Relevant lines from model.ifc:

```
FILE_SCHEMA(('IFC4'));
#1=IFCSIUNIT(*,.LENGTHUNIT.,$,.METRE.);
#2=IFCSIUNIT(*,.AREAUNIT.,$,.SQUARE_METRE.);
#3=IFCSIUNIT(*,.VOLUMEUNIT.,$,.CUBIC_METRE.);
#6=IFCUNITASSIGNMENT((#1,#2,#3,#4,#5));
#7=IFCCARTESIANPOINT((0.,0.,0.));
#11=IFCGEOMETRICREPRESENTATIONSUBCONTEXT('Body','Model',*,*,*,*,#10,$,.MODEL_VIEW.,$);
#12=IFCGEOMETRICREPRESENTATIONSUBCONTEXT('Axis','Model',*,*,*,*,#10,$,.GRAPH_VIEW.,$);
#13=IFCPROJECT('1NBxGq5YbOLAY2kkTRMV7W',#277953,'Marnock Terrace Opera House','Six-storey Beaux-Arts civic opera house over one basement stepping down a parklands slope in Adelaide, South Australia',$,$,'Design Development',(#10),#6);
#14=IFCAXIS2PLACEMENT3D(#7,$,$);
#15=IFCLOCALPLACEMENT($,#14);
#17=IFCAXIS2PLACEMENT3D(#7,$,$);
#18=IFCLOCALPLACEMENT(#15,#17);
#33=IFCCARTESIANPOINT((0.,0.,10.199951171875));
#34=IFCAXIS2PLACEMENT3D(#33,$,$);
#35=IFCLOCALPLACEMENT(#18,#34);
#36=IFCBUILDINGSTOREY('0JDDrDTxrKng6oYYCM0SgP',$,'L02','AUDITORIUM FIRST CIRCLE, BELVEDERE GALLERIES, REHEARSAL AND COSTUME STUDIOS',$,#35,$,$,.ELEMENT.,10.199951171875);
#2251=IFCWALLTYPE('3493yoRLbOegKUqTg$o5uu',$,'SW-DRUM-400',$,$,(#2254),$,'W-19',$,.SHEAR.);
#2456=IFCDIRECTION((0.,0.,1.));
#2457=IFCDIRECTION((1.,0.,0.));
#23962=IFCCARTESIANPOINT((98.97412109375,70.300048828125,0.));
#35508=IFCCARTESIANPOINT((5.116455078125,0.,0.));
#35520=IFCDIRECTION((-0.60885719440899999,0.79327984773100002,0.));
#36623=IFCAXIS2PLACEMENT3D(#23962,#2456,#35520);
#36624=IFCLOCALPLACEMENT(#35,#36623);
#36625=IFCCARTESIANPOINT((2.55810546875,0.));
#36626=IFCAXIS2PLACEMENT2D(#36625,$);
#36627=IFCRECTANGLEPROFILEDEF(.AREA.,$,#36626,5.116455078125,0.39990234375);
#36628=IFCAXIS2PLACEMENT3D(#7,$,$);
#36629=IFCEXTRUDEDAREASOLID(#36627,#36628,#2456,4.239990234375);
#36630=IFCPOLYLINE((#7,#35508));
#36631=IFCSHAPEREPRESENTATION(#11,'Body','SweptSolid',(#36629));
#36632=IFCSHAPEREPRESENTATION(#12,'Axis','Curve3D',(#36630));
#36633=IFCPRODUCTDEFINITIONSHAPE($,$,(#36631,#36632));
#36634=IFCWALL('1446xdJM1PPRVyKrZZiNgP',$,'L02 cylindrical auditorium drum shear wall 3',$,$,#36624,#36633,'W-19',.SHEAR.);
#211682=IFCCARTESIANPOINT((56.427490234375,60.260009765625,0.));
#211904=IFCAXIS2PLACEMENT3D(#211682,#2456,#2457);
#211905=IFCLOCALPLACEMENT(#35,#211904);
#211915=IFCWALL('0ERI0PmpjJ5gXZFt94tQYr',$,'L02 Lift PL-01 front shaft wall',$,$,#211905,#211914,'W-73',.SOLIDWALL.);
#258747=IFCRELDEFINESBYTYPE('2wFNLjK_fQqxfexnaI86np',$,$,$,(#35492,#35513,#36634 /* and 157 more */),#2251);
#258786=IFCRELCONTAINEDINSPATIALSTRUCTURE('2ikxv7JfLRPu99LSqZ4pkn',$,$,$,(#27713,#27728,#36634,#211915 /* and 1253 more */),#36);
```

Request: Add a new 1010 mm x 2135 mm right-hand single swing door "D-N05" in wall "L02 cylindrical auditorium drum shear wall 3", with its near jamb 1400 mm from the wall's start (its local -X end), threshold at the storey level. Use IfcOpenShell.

```python
import numpy as np
import ifcopenshell
import ifcopenshell.api.feature
import ifcopenshell.api.geometry
import ifcopenshell.api.root
import ifcopenshell.api.spatial
import ifcopenshell.geom
import ifcopenshell.util.element
import ifcopenshell.util.placement
import ifcopenshell.util.representation
import ifcopenshell.util.shape
import ifcopenshell.util.unit

model = ifcopenshell.open("model.ifc")
unit_scale = ifcopenshell.util.unit.calculate_unit_scale(model)
settings = ifcopenshell.geom.settings()


def volume(element):
    """Net volume in cubic metres, openings subtracted."""
    shape = ifcopenshell.geom.create_shape(settings, element)
    return ifcopenshell.util.shape.get_volume(shape.geometry)


wall = model.by_guid("1446xdJM1PPRVyKrZZiNgP")
storey = ifcopenshell.util.element.get_container(wall, ifc_class="IfcBuildingStorey")
context = ifcopenshell.util.representation.get_context(model, "Model", "Body", "MODEL_VIEW")
before = volume(wall)

width, height, from_end, sill = 1.01, 2.135, 1.4, 0.0  # metres

# The wall runs along its own X axis, and the end named is its -X end.
wall_shape = ifcopenshell.geom.create_shape(settings, wall)
x, y, z = ifcopenshell.util.shape.get_vertices(wall_shape.geometry).T
start = x.min() + from_end
face, thickness = float(y.min()), float(y.max() - y.min())
wall_matrix = ifcopenshell.util.placement.get_local_placement(wall.ObjectPlacement)
level = ifcopenshell.util.placement.get_local_placement(storey.ObjectPlacement)[2, 3]


def in_wall(x, y):
    """Placement at x, y metres in the wall's axes, at sill height."""
    matrix = wall_matrix.copy()
    matrix[:, 3] = wall_matrix @ np.array([x / unit_scale, y / unit_scale, 0.0, 1.0])
    matrix[2, 3] = level + sill / unit_scale
    return matrix


# Opening: a box that overshoots both wall faces by 50 mm.
opening = ifcopenshell.api.root.create_entity(model, ifc_class="IfcOpeningElement", predefined_type="OPENING")
box = ifcopenshell.api.geometry.add_wall_representation(
    model, context=context, length=width, height=height, thickness=thickness + 0.1
)
ifcopenshell.api.geometry.assign_representation(model, product=opening, representation=box)
ifcopenshell.api.geometry.edit_object_placement(model, product=opening, matrix=in_wall(start, face - 0.05), is_si=False)
ifcopenshell.api.feature.add_feature(model, feature=opening, element=wall)

door = ifcopenshell.api.root.create_entity(model, ifc_class="IfcDoor", name="D-N05", predefined_type="DOOR")
door.OverallWidth, door.OverallHeight = width / unit_scale, height / unit_scale
door.OperationType = "SINGLE_SWING_RIGHT"
body = ifcopenshell.api.geometry.add_door_representation(
    model,
    context=context,
    overall_width=door.OverallWidth,
    overall_height=door.OverallHeight,
    operation_type="SINGLE_SWING_RIGHT",
    lining_properties={"LiningDepth": thickness / unit_scale, "ThresholdDepth": thickness / unit_scale},
)
ifcopenshell.api.geometry.assign_representation(model, product=door, representation=body)
ifcopenshell.api.spatial.assign_container(model, products=[door], relating_structure=storey)
ifcopenshell.api.feature.add_filling(model, opening=opening, element=door)

# The lining spans the wall, so the door starts at the wall face.
ifcopenshell.api.geometry.edit_object_placement(model, product=door, matrix=in_wall(start, face), is_si=False)

after = volume(wall)

print(f"wall volume {before:.3f} -> {after:.3f} m3")

model.write("model_updated.ifc")
```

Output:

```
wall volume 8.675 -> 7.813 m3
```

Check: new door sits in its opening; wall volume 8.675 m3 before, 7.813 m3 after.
